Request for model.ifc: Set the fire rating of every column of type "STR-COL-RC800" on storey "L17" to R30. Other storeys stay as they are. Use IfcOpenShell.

First a look at what the model holds.

```python
import ifcopenshell
import ifcopenshell.util.element

model = ifcopenshell.open("model.ifc")
print(model.schema)
storey = next(s for s in model.by_type("IfcBuildingStorey") if s.Name == "L17")
columns = [e for e in ifcopenshell.util.element.get_decomposition(storey) if e.is_a("IfcColumn")]
seen = {}
for e in columns:
    element_type = ifcopenshell.util.element.get_type(e)
    key = (element_type.Name if element_type != e and element_type else None, ifcopenshell.util.element.get_pset(e, "Pset_ColumnCommon", "FireRating"))
    seen[key] = seen.get(key, 0) + 1
for (name, value), count in sorted(seen.items(), key=str):
    print(count, "x", name, "|", value)
```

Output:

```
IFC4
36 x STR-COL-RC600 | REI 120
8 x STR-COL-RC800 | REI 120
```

```python
import ifcopenshell
import ifcopenshell.api.pset
import ifcopenshell.util.element

model = ifcopenshell.open("model.ifc")

storey = next(s for s in model.by_type("IfcBuildingStorey") if s.Name == "L17")
columns = [e for e in ifcopenshell.util.element.get_decomposition(storey) if e.is_a("IfcColumn")]

count = 0
for e in columns:
    element_type = ifcopenshell.util.element.get_type(e)
    if element_type in (None, e) or element_type.Name != "STR-COL-RC800":
        continue
    # add_pset returns the element's existing set when there is one.
    pset = ifcopenshell.api.pset.add_pset(model, product=e, name="Pset_ColumnCommon")
    ifcopenshell.api.pset.edit_pset(model, pset=pset, properties={"FireRating": "R30"})
    count += 1

print(count, "columns updated")

model.write("model_edited.ifc")
```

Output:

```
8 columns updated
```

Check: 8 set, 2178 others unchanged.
